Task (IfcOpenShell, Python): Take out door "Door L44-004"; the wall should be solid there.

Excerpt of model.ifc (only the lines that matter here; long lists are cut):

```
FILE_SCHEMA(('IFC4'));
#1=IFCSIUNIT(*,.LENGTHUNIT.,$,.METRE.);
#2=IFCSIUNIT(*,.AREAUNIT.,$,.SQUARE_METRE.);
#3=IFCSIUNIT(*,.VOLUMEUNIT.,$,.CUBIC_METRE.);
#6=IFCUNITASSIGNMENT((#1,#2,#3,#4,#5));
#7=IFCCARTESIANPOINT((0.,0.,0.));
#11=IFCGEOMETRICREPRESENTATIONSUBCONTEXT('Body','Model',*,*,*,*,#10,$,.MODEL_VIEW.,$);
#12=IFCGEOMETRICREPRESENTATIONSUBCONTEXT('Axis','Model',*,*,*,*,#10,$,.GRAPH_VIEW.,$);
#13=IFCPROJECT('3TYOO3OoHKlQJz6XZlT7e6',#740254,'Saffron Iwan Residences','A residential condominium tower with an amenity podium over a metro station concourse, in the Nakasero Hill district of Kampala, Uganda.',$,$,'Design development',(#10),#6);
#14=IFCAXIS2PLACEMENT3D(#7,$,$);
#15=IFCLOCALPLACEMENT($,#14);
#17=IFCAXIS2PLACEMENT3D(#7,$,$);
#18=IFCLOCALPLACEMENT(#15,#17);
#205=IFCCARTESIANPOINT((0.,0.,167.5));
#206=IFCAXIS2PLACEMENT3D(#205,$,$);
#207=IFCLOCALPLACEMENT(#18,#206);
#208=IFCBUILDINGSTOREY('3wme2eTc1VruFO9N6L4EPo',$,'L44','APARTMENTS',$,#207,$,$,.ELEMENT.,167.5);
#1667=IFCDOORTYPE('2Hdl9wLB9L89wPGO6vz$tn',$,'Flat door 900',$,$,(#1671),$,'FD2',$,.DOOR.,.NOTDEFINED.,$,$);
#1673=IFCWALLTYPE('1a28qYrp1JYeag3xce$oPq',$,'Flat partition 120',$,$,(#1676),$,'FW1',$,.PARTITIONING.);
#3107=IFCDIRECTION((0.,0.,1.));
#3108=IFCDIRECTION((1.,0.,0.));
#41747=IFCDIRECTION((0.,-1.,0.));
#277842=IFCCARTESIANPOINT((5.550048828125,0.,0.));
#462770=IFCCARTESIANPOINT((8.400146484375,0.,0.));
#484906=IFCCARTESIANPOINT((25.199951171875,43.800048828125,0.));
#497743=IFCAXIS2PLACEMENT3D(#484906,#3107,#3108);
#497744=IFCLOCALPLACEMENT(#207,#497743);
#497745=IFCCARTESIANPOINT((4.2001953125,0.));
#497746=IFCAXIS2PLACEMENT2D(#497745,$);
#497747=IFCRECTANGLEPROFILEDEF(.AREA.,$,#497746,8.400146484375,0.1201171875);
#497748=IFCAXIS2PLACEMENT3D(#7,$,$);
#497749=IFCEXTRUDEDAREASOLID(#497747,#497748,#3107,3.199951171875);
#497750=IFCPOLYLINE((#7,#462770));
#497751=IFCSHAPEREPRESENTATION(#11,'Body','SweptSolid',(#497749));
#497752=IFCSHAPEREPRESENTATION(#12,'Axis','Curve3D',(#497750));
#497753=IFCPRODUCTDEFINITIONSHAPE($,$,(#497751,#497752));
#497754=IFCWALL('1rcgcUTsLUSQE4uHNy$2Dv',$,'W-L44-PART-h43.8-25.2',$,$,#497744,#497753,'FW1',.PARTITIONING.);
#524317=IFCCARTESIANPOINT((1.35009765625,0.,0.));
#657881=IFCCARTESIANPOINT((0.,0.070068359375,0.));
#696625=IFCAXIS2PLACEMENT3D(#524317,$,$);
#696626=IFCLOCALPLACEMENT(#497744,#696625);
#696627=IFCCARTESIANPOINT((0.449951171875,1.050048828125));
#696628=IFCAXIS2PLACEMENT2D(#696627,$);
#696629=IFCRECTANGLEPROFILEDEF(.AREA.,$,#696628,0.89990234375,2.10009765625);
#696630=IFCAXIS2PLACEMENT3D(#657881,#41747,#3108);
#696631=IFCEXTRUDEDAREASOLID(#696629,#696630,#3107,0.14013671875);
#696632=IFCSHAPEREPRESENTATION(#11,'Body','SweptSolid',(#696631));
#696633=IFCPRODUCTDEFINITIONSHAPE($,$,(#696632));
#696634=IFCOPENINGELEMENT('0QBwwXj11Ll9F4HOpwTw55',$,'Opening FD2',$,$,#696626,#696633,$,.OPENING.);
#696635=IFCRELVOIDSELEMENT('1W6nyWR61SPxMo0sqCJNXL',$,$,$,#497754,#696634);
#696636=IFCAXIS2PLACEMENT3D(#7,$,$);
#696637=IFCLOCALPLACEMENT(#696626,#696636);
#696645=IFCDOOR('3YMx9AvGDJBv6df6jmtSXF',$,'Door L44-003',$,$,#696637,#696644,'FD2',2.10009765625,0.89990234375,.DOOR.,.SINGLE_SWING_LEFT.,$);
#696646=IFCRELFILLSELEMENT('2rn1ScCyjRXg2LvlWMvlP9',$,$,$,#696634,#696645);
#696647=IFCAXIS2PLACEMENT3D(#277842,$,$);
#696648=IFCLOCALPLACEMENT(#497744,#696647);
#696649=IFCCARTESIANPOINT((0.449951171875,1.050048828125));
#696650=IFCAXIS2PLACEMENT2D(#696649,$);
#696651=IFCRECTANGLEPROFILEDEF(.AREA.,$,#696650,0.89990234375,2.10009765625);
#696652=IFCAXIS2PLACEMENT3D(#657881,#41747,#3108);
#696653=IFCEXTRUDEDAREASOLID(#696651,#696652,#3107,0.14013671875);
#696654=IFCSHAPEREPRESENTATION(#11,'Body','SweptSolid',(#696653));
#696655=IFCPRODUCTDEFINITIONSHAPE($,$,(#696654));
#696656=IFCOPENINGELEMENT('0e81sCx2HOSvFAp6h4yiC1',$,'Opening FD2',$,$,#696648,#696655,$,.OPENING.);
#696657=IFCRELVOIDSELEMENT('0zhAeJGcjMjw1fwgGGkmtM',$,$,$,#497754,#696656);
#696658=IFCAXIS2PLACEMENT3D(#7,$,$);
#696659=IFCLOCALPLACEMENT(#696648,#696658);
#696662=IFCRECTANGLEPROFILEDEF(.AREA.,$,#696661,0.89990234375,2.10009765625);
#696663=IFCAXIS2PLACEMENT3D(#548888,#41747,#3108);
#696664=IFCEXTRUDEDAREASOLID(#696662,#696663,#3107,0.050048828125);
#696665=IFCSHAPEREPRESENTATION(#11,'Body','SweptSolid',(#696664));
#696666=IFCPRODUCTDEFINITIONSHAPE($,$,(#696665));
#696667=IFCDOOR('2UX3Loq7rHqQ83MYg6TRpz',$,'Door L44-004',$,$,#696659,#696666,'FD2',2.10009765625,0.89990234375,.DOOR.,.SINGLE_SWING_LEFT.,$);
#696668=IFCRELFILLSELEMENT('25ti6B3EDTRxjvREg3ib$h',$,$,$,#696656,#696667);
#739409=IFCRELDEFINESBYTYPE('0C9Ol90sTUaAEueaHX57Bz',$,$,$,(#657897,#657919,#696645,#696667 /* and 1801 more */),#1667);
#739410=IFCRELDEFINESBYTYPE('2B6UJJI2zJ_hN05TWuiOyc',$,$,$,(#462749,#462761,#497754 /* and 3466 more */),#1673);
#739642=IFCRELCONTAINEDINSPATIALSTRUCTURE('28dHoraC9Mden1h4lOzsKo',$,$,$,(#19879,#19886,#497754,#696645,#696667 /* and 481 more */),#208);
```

```python
import ifcopenshell
import ifcopenshell.api.feature
import ifcopenshell.api.root
import ifcopenshell.geom
import ifcopenshell.util.shape

model = ifcopenshell.open("model.ifc")
settings = ifcopenshell.geom.settings()


def volume(element):
    """Net volume in cubic metres, openings subtracted."""
    shape = ifcopenshell.geom.create_shape(settings, element)
    return ifcopenshell.util.shape.get_volume(shape.geometry)


door = model.by_id(696667)
opening = door.FillsVoids[0].RelatingOpeningElement
wall = opening.VoidsElements[0].RelatingBuildingElement
before = volume(wall)

ifcopenshell.api.root.remove_product(model, product=door)
ifcopenshell.api.feature.remove_feature(model, feature=opening)

after = volume(wall)

print(f"wall volume {before:.3f} -> {after:.3f} m3")

model.write("model-out.ifc")
```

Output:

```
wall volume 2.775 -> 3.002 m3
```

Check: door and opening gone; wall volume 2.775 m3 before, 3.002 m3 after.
